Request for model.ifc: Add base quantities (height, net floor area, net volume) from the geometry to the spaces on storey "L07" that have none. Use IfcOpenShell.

First a look at what the model holds.

```python
import ifcopenshell
import ifcopenshell.util.element
import ifcopenshell.util.unit

model = ifcopenshell.open("model.ifc")
print(model.schema)
for unit_type in ("LENGTHUNIT", "AREAUNIT", "VOLUMEUNIT"):
    print(unit_type, ifcopenshell.util.unit.calculate_unit_scale(model, unit_type))
storey = next(s for s in model.by_type("IfcBuildingStorey") if s.Name == "L07")
spaces = [e for e in ifcopenshell.util.element.get_decomposition(storey) if e.is_a("IfcSpace")]
for e in sorted(spaces, key=lambda e: e.id()):
    print(e.id(), e.is_a(), e.Name, list(ifcopenshell.util.element.get_psets(e, qtos_only=True)), sep=" | ")
```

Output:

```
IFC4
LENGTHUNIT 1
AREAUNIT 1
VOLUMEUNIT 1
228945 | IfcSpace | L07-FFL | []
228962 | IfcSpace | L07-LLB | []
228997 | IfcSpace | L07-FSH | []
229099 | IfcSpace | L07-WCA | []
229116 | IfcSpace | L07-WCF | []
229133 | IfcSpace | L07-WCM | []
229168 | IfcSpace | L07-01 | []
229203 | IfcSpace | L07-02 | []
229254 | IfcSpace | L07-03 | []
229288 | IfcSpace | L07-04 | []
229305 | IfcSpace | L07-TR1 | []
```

```python
import ifcopenshell
import ifcopenshell.api.pset
import ifcopenshell.geom
import ifcopenshell.util.element
import ifcopenshell.util.shape
import ifcopenshell.util.unit

model = ifcopenshell.open("model.ifc")
unit_scale = ifcopenshell.util.unit.calculate_unit_scale(model)
area_scale = ifcopenshell.util.unit.calculate_unit_scale(model, "AREAUNIT")
volume_scale = ifcopenshell.util.unit.calculate_unit_scale(model, "VOLUMEUNIT")
settings = ifcopenshell.geom.settings()

storey = next(s for s in model.by_type("IfcBuildingStorey") if s.Name == "L07")
spaces = [e for e in ifcopenshell.util.element.get_decomposition(storey) if e.is_a("IfcSpace")]

for e in sorted(spaces, key=lambda e: e.id()):
    if ifcopenshell.util.element.get_psets(e, qtos_only=True, should_inherit=False):
        continue
    # Geometry comes back in metres, in the element's own axes.
    shape = ifcopenshell.geom.create_shape(settings, e)
    values = {
        "Height": ifcopenshell.util.shape.get_z(shape.geometry) / unit_scale,
        "NetFloorArea": ifcopenshell.util.shape.get_footprint_area(shape.geometry) / area_scale,
        "NetVolume": ifcopenshell.util.shape.get_volume(shape.geometry) / volume_scale,
    }
    qto = ifcopenshell.api.pset.add_qto(model, product=e, name="Qto_SpaceBaseQuantities")
    ifcopenshell.api.pset.edit_qto(model, qto=qto, properties=values)
    print(e.id(), {k: round(v, 3) for k, v in values.items()})

model.write("model_edited.ifc")
```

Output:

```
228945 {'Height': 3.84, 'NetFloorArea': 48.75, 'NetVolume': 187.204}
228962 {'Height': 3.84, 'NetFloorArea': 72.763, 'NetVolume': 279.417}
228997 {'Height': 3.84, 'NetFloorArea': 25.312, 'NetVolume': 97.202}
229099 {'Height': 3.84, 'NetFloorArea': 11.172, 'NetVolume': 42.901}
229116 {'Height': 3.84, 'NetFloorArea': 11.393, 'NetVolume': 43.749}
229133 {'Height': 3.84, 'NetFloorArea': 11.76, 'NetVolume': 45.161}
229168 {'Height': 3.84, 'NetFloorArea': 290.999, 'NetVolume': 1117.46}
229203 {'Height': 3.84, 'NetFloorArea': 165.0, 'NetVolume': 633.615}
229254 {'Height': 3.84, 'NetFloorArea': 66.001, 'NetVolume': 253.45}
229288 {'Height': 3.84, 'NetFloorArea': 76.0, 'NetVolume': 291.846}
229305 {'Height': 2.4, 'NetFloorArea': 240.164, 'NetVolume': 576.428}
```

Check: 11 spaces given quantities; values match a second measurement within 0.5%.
